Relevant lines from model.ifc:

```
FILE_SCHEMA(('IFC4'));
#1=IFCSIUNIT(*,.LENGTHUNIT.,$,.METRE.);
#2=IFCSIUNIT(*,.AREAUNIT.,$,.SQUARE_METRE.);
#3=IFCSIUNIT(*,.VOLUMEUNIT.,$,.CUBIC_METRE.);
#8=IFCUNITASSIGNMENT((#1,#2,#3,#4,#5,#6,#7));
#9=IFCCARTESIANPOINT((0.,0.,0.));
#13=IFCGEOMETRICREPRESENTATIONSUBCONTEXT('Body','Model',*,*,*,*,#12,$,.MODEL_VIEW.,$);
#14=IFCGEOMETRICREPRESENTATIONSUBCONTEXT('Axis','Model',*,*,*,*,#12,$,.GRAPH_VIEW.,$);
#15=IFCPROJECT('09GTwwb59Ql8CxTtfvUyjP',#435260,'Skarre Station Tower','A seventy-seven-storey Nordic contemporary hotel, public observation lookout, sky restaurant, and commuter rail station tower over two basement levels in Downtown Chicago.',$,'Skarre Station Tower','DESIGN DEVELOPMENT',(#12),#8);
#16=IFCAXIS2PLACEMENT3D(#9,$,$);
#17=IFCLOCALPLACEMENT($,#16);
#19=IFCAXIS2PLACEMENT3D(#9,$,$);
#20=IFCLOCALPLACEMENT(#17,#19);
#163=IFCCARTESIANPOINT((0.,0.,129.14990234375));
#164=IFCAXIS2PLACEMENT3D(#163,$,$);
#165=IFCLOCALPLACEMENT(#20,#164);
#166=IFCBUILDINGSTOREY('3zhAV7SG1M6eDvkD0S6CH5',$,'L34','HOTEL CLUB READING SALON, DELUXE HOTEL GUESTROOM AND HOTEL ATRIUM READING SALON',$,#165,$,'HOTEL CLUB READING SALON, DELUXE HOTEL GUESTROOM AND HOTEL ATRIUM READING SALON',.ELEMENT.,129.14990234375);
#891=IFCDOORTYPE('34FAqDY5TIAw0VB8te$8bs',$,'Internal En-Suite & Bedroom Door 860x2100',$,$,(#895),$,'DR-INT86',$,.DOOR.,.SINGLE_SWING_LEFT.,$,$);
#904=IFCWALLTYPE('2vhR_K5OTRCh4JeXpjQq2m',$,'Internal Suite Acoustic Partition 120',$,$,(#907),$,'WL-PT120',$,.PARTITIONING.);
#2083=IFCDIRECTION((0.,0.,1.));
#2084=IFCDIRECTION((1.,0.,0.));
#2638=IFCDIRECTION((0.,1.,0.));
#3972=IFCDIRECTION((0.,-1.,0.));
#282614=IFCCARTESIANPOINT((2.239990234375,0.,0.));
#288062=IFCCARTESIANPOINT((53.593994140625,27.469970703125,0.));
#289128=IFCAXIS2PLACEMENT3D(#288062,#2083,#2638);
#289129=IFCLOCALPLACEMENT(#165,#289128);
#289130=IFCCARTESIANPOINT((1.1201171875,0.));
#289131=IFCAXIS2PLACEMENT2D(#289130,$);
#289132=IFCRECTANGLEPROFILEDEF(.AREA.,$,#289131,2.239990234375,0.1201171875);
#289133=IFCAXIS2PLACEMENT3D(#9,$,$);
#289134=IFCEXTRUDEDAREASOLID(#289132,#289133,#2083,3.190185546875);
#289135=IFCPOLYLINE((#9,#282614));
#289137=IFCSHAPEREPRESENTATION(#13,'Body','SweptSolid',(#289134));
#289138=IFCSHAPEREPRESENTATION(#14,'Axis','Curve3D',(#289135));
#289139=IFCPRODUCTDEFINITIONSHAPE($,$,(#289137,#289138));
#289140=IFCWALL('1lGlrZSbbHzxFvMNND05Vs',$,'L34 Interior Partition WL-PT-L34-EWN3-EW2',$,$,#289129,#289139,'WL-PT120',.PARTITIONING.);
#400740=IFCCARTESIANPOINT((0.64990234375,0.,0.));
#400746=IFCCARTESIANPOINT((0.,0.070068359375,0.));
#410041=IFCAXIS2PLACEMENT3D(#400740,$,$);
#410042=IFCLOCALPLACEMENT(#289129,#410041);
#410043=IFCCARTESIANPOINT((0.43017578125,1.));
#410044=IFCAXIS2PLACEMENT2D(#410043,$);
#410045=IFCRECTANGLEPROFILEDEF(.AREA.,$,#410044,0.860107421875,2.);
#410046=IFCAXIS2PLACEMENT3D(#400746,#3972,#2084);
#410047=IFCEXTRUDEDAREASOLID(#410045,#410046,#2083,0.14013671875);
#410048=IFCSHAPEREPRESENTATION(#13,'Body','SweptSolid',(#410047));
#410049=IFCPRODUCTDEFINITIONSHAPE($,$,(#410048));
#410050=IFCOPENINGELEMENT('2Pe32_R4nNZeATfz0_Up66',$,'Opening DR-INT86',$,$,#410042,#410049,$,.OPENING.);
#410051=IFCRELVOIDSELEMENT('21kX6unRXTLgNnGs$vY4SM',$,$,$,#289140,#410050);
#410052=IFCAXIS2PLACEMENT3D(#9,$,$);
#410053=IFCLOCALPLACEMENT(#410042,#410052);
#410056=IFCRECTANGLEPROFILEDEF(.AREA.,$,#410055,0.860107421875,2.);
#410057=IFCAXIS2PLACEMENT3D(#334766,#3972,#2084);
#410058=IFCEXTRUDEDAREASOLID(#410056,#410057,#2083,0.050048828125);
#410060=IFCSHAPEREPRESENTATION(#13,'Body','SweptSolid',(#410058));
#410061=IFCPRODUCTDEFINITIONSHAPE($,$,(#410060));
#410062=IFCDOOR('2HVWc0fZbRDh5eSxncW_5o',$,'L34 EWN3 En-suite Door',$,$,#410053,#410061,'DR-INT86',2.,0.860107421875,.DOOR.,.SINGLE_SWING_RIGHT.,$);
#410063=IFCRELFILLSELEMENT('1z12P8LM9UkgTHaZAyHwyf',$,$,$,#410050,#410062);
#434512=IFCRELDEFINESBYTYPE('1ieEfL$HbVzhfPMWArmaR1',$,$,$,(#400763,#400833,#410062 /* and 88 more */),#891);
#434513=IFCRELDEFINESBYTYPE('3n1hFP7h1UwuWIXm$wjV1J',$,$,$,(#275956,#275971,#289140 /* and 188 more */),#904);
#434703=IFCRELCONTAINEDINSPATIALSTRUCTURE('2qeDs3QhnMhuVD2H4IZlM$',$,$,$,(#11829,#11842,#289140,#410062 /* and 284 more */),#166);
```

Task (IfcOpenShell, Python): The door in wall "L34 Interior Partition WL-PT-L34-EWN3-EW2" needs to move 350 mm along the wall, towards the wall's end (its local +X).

```python
import ifcopenshell
import ifcopenshell.api.geometry
import ifcopenshell.util.placement
import ifcopenshell.util.unit

model = ifcopenshell.open("model.ifc")
unit_scale = ifcopenshell.util.unit.calculate_unit_scale(model)

door = model.by_guid("2HVWc0fZbRDh5eSxncW_5o")
opening = door.FillsVoids[0].RelatingOpeningElement
wall = opening.VoidsElements[0].RelatingBuildingElement

wall_matrix = ifcopenshell.util.placement.get_local_placement(wall.ObjectPlacement)
shift = wall_matrix[:3, 0] * 0.35 / unit_scale
before = ifcopenshell.util.placement.get_local_placement(door.ObjectPlacement)[:3, 3].copy()

# The door is placed relative to its opening, so it follows when the opening moves.
matrix = ifcopenshell.util.placement.get_local_placement(opening.ObjectPlacement)
matrix[:3, 3] += shift
ifcopenshell.api.geometry.edit_object_placement(
    model, product=opening, matrix=matrix, is_si=False, should_transform_children=True
)

after = ifcopenshell.util.placement.get_local_placement(door.ObjectPlacement)[:3, 3]
print("door moved by", (after - before).round(3) + 0.0)

model.write("model_edited.ifc")
```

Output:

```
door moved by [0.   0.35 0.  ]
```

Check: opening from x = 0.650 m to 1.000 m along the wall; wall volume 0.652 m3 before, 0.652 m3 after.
